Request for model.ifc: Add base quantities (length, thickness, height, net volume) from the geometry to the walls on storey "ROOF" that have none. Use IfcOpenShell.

First a look at what the model holds.

```python
import ifcopenshell
import ifcopenshell.util.element
import ifcopenshell.util.unit

model = ifcopenshell.open("model.ifc")
print(model.schema)
for unit_type in ("LENGTHUNIT", "AREAUNIT", "VOLUMEUNIT"):
    print(unit_type, ifcopenshell.util.unit.calculate_unit_scale(model, unit_type))
storey = next(s for s in model.by_type("IfcBuildingStorey") if s.Name == "ROOF")
walls = [e for e in ifcopenshell.util.element.get_decomposition(storey) if e.is_a("IfcWall")]
for e in sorted(walls, key=lambda e: e.id()):
    print(e.id(), e.is_a(), e.Name, list(ifcopenshell.util.element.get_psets(e, qtos_only=True)), sep=" | ")
```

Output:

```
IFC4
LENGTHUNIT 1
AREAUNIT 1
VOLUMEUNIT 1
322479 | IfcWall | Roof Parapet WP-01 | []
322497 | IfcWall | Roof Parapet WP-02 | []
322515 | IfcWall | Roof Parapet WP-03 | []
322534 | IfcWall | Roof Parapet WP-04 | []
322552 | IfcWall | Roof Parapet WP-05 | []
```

```python
import ifcopenshell
import ifcopenshell.api.pset
import ifcopenshell.geom
import ifcopenshell.util.element
import ifcopenshell.util.shape
import ifcopenshell.util.unit

model = ifcopenshell.open("model.ifc")
unit_scale = ifcopenshell.util.unit.calculate_unit_scale(model)
volume_scale = ifcopenshell.util.unit.calculate_unit_scale(model, "VOLUMEUNIT")
settings = ifcopenshell.geom.settings()

storey = next(s for s in model.by_type("IfcBuildingStorey") if s.Name == "ROOF")
walls = [e for e in ifcopenshell.util.element.get_decomposition(storey) if e.is_a("IfcWall")]

for e in sorted(walls, key=lambda e: e.id()):
    if ifcopenshell.util.element.get_psets(e, qtos_only=True, should_inherit=False):
        continue
    # Geometry comes back in metres, in the element's own axes.
    shape = ifcopenshell.geom.create_shape(settings, e)
    values = {
        "Length": ifcopenshell.util.shape.get_x(shape.geometry) / unit_scale,
        "Width": ifcopenshell.util.shape.get_y(shape.geometry) / unit_scale,
        "Height": ifcopenshell.util.shape.get_z(shape.geometry) / unit_scale,
        "NetVolume": ifcopenshell.util.shape.get_volume(shape.geometry) / volume_scale,
    }
    qto = ifcopenshell.api.pset.add_qto(model, product=e, name="Qto_WallBaseQuantities")
    ifcopenshell.api.pset.edit_qto(model, qto=qto, properties=values)
    print(e.id(), {k: round(v, 3) for k, v in values.items()})

model.write("model_v2.ifc")
```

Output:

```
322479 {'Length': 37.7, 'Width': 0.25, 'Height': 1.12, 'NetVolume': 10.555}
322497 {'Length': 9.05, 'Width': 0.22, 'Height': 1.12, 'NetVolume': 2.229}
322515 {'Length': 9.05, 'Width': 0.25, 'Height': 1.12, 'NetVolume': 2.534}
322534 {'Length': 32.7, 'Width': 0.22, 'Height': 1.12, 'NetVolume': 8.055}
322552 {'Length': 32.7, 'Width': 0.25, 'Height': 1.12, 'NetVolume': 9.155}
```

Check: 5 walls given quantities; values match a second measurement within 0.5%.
